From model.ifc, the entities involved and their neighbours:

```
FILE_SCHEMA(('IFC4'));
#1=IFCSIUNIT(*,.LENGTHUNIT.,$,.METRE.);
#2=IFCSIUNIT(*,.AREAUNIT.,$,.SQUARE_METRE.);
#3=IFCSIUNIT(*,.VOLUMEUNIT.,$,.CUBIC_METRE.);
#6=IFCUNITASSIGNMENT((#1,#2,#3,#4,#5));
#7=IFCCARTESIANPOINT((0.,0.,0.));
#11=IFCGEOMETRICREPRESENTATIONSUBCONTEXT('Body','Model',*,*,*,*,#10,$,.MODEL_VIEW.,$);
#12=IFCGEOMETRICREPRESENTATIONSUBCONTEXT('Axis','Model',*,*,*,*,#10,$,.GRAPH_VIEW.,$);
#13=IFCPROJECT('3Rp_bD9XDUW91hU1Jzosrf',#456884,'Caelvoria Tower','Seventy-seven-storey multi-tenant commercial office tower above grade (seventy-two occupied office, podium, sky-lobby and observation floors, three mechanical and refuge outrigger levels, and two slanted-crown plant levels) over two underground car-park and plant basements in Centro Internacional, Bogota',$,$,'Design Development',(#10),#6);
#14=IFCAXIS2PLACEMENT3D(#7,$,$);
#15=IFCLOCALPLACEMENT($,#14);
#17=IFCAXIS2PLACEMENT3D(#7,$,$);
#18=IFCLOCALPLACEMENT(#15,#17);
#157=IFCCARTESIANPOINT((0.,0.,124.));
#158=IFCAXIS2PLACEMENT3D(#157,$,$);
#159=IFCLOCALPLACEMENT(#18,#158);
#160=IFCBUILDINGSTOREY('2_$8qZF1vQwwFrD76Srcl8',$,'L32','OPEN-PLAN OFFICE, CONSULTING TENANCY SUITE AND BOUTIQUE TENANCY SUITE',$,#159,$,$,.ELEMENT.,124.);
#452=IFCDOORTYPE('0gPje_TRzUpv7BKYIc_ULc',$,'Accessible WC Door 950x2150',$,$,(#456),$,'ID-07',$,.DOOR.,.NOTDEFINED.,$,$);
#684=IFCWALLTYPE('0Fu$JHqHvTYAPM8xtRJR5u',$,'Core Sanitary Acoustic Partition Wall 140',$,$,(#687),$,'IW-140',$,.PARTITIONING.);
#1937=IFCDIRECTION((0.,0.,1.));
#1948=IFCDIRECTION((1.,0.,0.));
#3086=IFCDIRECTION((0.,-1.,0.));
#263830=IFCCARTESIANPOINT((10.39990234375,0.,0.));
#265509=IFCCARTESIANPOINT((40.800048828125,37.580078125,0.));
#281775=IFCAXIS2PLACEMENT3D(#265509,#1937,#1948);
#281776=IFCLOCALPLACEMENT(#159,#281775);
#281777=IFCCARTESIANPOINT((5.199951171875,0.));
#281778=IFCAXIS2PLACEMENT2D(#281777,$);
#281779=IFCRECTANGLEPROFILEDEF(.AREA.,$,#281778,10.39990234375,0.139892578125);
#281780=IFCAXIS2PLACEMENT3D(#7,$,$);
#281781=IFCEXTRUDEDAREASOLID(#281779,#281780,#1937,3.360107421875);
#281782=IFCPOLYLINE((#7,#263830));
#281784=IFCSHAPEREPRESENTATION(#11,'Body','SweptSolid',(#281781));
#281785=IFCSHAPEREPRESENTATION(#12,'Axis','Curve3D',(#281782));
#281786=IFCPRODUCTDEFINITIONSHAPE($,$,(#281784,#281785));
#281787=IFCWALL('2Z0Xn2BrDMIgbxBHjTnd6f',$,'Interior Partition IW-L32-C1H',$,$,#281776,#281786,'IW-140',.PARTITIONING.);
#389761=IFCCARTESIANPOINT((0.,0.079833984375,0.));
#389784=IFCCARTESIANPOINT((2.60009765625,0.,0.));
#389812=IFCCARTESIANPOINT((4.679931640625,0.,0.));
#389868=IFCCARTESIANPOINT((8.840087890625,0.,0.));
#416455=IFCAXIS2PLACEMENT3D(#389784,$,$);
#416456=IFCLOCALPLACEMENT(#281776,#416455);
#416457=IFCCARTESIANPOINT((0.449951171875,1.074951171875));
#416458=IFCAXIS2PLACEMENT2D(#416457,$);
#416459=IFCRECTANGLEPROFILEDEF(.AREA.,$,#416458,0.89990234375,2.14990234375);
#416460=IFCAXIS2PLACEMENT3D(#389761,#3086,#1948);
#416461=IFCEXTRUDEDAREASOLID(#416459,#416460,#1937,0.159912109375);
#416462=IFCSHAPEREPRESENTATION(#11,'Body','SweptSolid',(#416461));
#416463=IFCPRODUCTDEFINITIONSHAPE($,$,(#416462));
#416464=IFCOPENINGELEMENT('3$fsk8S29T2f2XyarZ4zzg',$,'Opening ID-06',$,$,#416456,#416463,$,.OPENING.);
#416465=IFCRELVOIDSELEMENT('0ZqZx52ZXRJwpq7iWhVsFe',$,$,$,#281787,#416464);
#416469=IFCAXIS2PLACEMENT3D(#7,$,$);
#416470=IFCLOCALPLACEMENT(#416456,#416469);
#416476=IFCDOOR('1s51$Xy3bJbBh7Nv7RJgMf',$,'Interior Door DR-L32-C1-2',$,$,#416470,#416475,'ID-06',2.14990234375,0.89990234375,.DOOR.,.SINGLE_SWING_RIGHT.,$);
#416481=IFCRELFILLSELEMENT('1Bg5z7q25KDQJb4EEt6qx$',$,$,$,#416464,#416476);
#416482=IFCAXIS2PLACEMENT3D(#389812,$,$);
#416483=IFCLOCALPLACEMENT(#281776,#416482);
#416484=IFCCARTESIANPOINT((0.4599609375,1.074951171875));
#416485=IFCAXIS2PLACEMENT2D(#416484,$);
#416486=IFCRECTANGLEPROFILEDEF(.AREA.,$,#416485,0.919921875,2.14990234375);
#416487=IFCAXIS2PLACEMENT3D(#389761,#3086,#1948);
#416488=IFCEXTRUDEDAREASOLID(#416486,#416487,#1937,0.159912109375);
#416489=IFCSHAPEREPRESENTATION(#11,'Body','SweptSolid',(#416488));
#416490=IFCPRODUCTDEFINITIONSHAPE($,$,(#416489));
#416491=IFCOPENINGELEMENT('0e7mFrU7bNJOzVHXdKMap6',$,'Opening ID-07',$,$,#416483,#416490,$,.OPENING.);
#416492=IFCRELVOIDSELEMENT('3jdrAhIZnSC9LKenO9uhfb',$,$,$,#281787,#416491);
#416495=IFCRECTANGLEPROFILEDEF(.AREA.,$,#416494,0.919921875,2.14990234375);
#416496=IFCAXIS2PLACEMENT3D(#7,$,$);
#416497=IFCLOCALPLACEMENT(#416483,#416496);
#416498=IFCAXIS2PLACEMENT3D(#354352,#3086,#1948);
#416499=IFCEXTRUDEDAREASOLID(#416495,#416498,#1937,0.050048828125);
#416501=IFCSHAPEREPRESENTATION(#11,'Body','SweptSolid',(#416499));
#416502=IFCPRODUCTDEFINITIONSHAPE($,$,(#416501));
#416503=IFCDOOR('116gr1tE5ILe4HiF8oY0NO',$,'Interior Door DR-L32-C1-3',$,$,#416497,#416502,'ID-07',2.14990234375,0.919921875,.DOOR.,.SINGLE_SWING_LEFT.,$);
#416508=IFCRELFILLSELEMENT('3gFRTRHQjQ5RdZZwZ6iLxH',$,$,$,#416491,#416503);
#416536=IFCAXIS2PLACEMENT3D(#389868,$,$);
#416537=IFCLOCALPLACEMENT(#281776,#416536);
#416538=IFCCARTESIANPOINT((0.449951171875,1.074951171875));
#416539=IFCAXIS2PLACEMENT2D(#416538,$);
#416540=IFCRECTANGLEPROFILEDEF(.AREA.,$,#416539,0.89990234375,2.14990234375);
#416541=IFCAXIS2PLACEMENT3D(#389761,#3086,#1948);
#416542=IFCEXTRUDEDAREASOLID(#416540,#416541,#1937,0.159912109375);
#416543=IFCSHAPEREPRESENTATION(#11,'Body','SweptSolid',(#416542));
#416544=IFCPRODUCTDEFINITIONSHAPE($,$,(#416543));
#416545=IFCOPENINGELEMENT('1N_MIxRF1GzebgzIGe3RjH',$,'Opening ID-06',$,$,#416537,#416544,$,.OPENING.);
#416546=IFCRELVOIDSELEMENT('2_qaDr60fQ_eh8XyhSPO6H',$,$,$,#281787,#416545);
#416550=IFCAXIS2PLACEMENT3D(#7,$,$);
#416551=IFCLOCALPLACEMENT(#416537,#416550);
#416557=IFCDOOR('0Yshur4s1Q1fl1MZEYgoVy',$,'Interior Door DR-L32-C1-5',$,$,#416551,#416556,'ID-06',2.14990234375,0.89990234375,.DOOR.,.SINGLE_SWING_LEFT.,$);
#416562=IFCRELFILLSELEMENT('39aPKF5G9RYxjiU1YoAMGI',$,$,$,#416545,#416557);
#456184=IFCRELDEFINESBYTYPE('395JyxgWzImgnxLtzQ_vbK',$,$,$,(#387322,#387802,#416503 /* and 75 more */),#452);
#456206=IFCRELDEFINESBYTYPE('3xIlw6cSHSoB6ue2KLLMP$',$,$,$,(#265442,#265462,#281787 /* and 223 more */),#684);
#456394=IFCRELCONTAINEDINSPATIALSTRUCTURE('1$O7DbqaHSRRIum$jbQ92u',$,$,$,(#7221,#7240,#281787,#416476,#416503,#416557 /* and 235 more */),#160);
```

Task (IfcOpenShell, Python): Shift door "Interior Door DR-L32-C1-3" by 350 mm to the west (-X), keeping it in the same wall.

```python
import ifcopenshell
import ifcopenshell.api.geometry
import ifcopenshell.util.placement
import ifcopenshell.util.unit

model = ifcopenshell.open("model.ifc")
unit_scale = ifcopenshell.util.unit.calculate_unit_scale(model)

door = model.by_guid("116gr1tE5ILe4HiF8oY0NO")
opening = door.FillsVoids[0].RelatingOpeningElement
wall = opening.VoidsElements[0].RelatingBuildingElement

wall_matrix = ifcopenshell.util.placement.get_local_placement(wall.ObjectPlacement)
shift = wall_matrix[:3, 0] * -0.35 / unit_scale
before = ifcopenshell.util.placement.get_local_placement(door.ObjectPlacement)[:3, 3].copy()

# The door is placed relative to its opening, so it follows when the opening moves.
matrix = ifcopenshell.util.placement.get_local_placement(opening.ObjectPlacement)
matrix[:3, 3] += shift
ifcopenshell.api.geometry.edit_object_placement(
    model, product=opening, matrix=matrix, is_si=False, should_transform_children=True
)

after = ifcopenshell.util.placement.get_local_placement(door.ObjectPlacement)[:3, 3]
print("door moved by", (after - before).round(3) + 0.0)

model.write("model_v2.ifc")
```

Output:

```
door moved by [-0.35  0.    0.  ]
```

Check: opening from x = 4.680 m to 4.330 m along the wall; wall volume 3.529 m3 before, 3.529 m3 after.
